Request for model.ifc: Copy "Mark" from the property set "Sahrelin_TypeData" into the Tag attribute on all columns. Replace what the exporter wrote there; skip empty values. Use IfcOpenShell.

First a look at what the model holds.

```python
import ifcopenshell
import ifcopenshell.util.element

model = ifcopenshell.open("model.ifc")
print(model.schema)
columns = model.by_type("IfcColumn")
print(len(columns), "columns")
for e in columns[:8]:
    source = ifcopenshell.util.element.get_pset(e, "Sahrelin_TypeData", "Mark")
    target = e.Tag
    print(e.id(), repr(source), repr(target), sep=" | ")
```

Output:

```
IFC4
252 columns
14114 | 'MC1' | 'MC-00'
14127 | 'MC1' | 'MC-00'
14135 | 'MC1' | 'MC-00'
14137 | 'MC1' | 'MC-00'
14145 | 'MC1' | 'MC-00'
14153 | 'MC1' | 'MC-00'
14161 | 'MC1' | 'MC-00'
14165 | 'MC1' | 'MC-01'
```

```python
import ifcopenshell
import ifcopenshell.util.element

model = ifcopenshell.open("model.ifc")

count = 0
for e in model.by_type("IfcColumn"):
    value = ifcopenshell.util.element.get_pset(e, "Sahrelin_TypeData", "Mark")
    current = e.Tag
    if not value or not value.strip() or current == value:
        continue
    e.Tag = value
    count += 1

print(count, "columns updated")

model.write("model_edited.ifc")
```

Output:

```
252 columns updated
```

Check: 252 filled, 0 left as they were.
